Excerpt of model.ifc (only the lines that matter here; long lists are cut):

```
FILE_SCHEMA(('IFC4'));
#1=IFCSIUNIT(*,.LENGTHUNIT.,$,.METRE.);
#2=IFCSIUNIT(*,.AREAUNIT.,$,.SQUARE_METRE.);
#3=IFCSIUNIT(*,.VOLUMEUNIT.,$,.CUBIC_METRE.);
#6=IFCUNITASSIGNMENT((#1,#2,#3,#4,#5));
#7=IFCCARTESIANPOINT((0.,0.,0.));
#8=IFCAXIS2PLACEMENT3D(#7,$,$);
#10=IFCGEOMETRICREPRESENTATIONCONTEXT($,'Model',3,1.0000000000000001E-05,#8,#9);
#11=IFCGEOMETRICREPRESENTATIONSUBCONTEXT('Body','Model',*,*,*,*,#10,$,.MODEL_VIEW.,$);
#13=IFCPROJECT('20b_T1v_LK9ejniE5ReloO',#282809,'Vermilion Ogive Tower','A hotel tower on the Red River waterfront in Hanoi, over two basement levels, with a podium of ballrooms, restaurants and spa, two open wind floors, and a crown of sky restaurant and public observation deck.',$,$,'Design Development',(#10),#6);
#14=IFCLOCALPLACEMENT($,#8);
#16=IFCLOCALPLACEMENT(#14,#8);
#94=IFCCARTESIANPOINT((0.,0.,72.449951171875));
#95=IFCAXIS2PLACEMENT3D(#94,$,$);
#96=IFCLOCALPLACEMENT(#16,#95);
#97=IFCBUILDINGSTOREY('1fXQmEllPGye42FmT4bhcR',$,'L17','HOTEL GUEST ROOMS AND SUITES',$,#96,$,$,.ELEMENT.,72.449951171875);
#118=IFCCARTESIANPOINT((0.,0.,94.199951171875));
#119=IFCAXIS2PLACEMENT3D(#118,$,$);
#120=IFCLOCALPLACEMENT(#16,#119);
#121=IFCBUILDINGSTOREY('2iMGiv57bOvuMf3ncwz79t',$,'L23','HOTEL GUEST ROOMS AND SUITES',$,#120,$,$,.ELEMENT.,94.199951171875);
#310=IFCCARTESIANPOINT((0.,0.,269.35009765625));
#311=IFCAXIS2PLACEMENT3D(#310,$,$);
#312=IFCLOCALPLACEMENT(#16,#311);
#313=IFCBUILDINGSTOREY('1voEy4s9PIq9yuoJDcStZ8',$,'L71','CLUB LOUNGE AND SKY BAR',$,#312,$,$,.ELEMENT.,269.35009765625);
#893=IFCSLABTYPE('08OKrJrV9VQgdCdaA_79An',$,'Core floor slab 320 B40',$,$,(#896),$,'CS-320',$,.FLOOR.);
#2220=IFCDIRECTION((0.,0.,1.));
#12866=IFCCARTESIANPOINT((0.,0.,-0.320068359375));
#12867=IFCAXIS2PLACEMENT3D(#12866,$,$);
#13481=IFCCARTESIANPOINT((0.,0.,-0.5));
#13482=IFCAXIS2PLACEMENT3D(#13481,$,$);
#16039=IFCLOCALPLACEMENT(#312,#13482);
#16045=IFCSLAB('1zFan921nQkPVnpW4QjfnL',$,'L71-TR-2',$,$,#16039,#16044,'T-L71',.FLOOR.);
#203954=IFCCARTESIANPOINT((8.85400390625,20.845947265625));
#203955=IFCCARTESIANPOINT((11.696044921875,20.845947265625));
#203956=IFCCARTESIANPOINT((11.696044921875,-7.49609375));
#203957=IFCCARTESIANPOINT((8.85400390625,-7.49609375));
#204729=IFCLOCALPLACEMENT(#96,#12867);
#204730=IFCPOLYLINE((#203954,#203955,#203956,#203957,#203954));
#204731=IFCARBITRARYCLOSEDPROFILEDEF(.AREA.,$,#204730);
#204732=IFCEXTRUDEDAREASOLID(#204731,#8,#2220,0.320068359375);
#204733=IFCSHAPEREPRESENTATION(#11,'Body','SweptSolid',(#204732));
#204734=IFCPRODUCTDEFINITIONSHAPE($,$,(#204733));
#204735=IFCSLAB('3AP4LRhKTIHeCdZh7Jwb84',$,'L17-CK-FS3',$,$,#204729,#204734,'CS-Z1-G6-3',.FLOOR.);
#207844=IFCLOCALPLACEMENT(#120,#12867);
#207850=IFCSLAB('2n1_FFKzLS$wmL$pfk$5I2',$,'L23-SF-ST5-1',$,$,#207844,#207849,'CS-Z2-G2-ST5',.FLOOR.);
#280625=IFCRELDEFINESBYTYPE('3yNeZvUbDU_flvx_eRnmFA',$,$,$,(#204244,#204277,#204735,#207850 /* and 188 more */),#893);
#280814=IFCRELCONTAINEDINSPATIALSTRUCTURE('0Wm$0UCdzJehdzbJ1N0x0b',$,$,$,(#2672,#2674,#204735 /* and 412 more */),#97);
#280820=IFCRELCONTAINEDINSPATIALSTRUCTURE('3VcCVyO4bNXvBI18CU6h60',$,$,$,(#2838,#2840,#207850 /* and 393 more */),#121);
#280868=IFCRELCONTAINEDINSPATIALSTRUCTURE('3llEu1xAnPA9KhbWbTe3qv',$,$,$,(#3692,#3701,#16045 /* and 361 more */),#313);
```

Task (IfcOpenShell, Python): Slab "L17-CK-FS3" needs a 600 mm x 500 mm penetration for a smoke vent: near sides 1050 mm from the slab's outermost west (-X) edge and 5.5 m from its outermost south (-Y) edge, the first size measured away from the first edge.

```python
import numpy as np
import ifcopenshell
import ifcopenshell.api.feature
import ifcopenshell.api.geometry
import ifcopenshell.api.root
import ifcopenshell.geom
import ifcopenshell.util.placement
import ifcopenshell.util.representation
import ifcopenshell.util.shape
import ifcopenshell.util.unit

model = ifcopenshell.open("model.ifc")
unit_scale = ifcopenshell.util.unit.calculate_unit_scale(model)
settings = ifcopenshell.geom.settings()


def volume(element):
    """Net volume in cubic metres, openings subtracted."""
    shape = ifcopenshell.geom.create_shape(settings, element)
    return ifcopenshell.util.shape.get_volume(shape.geometry)


slab = model.by_guid("3AP4LRhKTIHeCdZh7Jwb84")
before = volume(slab)

# Extent in the slab's own axes, in metres. The edges named are its -X and -Y sides.
slab_shape = ifcopenshell.geom.create_shape(settings, slab)
vertices = ifcopenshell.util.shape.get_vertices(slab_shape.geometry)
x_min, y_min, bottom = vertices.min(axis=0)
top = vertices[:, 2].max()

opening = ifcopenshell.api.root.create_entity(model, ifc_class="IfcOpeningElement", name="Smoke vent opening", predefined_type="OPENING")
context = ifcopenshell.util.representation.get_context(model, "Model", "Body", "MODEL_VIEW")
width, depth = 0.6, 0.5
outline = [(0.0, 0.0), (width, 0.0), (width, depth), (0.0, depth), (0.0, 0.0)]
# Overshoot both faces by 50 mm so the cut is clean.
shape = ifcopenshell.api.geometry.add_slab_representation(
    model, context=context, depth=top - bottom + 0.1, polyline=outline
)
ifcopenshell.api.geometry.assign_representation(model, product=opening, representation=shape)

matrix = ifcopenshell.util.placement.get_local_placement(slab.ObjectPlacement)
matrix[:, 3] = matrix @ np.append(np.array([x_min + 1.05, y_min + 5.5, bottom - 0.05]) / unit_scale, 1.0)
ifcopenshell.api.geometry.edit_object_placement(model, product=opening, matrix=matrix, is_si=False)
ifcopenshell.api.feature.add_feature(model, feature=opening, element=slab)

after = volume(slab)

print(f"slab volume {before:.3f} -> {after:.3f} m3")

model.write("model_updated.ifc")
```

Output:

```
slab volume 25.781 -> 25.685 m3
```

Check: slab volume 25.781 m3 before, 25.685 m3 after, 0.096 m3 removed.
